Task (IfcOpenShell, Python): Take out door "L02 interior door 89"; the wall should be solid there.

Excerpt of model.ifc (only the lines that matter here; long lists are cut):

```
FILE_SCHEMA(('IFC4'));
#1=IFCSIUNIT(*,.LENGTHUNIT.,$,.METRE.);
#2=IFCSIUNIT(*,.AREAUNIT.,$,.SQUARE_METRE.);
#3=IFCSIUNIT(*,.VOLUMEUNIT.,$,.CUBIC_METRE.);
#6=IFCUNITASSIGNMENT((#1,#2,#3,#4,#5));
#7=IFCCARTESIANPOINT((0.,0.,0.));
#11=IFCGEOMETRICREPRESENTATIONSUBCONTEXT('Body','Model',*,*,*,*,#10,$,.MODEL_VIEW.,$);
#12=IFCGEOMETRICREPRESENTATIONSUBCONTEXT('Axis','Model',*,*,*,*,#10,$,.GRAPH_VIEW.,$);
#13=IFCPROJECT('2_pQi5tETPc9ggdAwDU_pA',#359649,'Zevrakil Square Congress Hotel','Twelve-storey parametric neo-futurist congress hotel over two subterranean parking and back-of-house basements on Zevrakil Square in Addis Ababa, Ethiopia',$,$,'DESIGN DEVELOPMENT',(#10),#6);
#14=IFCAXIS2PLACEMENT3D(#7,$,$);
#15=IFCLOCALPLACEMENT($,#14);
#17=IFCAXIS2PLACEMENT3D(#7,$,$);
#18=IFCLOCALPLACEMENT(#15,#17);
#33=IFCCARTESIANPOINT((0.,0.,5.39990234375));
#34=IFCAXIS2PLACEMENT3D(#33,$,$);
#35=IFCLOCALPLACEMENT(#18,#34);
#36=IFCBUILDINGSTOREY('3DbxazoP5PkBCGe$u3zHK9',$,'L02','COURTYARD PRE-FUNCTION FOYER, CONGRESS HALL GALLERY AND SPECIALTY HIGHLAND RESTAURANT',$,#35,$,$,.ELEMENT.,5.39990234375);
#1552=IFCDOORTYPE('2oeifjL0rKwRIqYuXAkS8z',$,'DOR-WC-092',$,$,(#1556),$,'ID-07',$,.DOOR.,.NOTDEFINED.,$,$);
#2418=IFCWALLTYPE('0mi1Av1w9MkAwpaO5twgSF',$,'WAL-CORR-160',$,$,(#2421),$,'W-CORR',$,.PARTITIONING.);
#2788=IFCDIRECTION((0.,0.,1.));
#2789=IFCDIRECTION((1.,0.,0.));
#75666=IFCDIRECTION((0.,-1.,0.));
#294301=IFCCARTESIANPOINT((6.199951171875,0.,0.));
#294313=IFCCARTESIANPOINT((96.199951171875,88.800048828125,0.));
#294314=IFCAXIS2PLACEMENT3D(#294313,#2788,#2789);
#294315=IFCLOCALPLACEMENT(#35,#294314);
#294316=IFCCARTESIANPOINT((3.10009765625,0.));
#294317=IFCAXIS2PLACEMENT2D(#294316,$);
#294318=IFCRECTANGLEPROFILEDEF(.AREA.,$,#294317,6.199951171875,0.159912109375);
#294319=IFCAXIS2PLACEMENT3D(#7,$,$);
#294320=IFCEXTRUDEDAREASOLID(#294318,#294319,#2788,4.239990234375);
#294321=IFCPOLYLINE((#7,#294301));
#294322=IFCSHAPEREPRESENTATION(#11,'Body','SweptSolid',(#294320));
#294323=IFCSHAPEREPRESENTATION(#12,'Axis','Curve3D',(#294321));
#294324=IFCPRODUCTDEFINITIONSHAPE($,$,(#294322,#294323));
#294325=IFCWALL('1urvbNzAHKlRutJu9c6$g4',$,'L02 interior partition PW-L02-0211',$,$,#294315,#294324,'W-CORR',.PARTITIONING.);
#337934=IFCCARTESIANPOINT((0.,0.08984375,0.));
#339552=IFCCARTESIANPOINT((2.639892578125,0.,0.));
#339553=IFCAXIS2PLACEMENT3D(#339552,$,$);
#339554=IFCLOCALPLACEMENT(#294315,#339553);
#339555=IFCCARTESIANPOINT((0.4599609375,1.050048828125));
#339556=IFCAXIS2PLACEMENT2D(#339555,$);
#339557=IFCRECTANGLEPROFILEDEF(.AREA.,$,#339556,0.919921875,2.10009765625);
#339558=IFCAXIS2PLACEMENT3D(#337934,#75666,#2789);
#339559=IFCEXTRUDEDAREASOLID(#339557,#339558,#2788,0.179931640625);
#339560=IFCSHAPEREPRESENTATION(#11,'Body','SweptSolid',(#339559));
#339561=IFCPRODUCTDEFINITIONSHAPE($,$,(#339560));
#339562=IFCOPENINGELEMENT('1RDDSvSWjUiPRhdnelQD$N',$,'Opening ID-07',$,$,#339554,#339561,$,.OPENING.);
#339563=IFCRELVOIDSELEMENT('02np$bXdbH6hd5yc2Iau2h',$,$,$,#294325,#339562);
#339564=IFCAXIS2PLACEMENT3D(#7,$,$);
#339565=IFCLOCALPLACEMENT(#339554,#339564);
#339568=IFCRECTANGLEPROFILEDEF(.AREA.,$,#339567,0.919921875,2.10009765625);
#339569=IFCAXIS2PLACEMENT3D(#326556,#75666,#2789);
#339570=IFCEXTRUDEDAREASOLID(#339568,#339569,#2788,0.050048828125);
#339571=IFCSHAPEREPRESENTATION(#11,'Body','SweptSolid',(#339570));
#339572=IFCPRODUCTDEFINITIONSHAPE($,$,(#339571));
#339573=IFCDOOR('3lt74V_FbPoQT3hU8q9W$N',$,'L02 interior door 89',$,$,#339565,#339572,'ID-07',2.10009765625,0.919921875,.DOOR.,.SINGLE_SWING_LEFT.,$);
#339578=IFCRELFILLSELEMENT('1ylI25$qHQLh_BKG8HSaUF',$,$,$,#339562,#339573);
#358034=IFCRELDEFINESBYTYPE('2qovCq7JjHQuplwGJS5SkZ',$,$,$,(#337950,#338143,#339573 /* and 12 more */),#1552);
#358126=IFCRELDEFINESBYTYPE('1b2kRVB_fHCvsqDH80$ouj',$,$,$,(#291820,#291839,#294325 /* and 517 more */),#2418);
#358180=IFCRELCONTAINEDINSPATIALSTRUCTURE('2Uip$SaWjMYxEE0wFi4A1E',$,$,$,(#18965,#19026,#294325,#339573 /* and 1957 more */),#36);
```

```python
import ifcopenshell
import ifcopenshell.api.feature
import ifcopenshell.api.root
import ifcopenshell.geom
import ifcopenshell.util.shape

model = ifcopenshell.open("model.ifc")
settings = ifcopenshell.geom.settings()


def volume(element):
    """Net volume in cubic metres, openings subtracted."""
    shape = ifcopenshell.geom.create_shape(settings, element)
    return ifcopenshell.util.shape.get_volume(shape.geometry)


door = model.by_guid("3lt74V_FbPoQT3hU8q9W$N")
opening = door.FillsVoids[0].RelatingOpeningElement
wall = opening.VoidsElements[0].RelatingBuildingElement
before = volume(wall)

ifcopenshell.api.root.remove_product(model, product=door)
ifcopenshell.api.feature.remove_feature(model, feature=opening)

after = volume(wall)

print(f"wall volume {before:.3f} -> {after:.3f} m3")

model.write("model_updated.ifc")
```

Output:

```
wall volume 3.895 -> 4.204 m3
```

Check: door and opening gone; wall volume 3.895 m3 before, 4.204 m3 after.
